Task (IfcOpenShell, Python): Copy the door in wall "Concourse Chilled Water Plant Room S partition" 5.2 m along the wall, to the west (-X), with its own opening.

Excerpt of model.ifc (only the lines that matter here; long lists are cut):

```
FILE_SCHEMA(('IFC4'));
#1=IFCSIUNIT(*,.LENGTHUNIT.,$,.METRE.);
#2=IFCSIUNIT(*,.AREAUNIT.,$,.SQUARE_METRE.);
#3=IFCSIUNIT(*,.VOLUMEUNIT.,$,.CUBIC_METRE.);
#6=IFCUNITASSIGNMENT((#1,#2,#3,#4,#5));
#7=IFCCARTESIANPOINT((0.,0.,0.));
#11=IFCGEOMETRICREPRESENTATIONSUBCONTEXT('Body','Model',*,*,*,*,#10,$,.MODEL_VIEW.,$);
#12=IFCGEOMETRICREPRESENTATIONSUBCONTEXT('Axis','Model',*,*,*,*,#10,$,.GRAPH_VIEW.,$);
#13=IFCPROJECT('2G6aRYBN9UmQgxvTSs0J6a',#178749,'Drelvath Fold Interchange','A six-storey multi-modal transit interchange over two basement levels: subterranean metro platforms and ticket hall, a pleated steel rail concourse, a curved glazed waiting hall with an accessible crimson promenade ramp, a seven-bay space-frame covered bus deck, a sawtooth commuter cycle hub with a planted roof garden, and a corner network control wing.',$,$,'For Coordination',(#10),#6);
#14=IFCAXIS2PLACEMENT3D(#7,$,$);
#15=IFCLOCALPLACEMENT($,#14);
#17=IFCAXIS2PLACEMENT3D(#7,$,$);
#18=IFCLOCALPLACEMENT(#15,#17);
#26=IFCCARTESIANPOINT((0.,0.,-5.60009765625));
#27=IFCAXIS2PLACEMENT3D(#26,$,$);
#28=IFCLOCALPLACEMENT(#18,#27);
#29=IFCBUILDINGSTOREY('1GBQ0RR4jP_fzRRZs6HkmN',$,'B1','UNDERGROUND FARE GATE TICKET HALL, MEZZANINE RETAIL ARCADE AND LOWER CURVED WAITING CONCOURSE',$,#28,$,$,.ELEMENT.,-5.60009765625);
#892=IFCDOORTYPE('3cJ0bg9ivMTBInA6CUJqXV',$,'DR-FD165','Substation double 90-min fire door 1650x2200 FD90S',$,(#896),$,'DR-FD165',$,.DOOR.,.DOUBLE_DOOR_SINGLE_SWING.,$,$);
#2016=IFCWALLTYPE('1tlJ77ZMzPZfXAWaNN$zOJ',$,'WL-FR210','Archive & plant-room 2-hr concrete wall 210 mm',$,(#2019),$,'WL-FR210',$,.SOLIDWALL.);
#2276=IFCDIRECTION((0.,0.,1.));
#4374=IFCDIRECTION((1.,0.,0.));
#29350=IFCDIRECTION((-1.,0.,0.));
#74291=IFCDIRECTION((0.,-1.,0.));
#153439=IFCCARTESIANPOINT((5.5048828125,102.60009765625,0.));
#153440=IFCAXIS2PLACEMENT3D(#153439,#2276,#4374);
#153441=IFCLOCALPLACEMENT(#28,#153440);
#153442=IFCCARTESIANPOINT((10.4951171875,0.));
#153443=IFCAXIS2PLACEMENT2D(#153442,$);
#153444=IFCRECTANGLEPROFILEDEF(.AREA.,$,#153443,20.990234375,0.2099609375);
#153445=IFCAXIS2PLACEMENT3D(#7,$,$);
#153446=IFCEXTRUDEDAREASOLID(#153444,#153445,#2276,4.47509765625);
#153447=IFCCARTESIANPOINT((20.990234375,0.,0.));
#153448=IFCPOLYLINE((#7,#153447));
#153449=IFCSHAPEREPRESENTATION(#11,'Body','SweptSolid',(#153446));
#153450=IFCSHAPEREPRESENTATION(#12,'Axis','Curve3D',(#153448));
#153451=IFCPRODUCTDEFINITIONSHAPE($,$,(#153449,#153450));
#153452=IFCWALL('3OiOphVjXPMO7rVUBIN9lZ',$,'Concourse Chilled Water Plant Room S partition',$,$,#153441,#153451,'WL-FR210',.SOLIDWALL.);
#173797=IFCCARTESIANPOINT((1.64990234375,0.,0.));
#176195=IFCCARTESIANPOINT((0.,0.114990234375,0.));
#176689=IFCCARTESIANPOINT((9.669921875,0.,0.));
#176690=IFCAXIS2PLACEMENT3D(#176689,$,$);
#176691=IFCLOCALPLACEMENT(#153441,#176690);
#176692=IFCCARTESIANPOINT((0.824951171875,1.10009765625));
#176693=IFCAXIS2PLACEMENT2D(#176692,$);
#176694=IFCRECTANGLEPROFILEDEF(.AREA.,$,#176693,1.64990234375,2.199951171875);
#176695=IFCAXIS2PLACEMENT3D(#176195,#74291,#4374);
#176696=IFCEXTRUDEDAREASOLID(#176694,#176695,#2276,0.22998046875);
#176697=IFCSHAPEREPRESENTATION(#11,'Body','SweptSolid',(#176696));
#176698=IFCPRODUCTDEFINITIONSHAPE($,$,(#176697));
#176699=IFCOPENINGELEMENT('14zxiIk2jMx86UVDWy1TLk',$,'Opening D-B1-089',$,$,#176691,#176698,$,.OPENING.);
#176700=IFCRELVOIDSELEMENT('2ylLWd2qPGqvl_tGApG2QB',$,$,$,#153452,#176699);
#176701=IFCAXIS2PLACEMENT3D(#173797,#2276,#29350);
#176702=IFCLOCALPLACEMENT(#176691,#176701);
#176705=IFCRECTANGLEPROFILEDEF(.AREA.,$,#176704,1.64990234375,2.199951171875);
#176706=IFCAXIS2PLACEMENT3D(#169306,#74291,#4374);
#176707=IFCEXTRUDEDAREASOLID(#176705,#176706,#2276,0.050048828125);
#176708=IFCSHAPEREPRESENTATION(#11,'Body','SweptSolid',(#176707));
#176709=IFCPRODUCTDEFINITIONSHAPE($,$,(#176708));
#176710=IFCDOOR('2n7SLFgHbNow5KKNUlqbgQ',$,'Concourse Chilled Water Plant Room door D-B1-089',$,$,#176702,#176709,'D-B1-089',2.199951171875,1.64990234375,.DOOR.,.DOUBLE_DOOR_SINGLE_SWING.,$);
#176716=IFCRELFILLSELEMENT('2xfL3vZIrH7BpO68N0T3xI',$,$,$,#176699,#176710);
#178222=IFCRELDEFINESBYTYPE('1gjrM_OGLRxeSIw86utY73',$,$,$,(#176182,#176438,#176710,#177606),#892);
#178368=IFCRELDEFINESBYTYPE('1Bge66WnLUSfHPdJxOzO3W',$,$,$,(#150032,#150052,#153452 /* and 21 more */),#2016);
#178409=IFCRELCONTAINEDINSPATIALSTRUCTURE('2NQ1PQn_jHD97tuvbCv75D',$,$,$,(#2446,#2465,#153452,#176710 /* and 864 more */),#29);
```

```python
import ifcopenshell
import ifcopenshell.api.feature
import ifcopenshell.api.geometry
import ifcopenshell.api.root
import ifcopenshell.geom
import ifcopenshell.util.element
import ifcopenshell.util.placement
import ifcopenshell.util.shape
import ifcopenshell.util.unit

model = ifcopenshell.open("model.ifc")
unit_scale = ifcopenshell.util.unit.calculate_unit_scale(model)
settings = ifcopenshell.geom.settings()


def volume(element):
    """Net volume in cubic metres, openings subtracted."""
    shape = ifcopenshell.geom.create_shape(settings, element)
    return ifcopenshell.util.shape.get_volume(shape.geometry)


door = model.by_guid("2n7SLFgHbNow5KKNUlqbgQ")
opening = door.FillsVoids[0].RelatingOpeningElement
wall = opening.VoidsElements[0].RelatingBuildingElement
before = volume(wall)
shift = ifcopenshell.util.placement.get_local_placement(wall.ObjectPlacement)[:3, 0] * -5.2 / unit_scale

# copy_class copies the void relationship, type, container and properties, but no geometry.
new_opening = ifcopenshell.api.root.copy_class(model, product=opening)
new_opening.Representation = ifcopenshell.util.element.copy_deep(
    model, opening.Representation, exclude=["IfcGeometricRepresentationContext", "IfcRepresentationMap"]
)
new_door = ifcopenshell.api.root.copy_class(model, product=door)
new_door.Representation = ifcopenshell.util.element.copy_deep(
    model, door.Representation, exclude=["IfcGeometricRepresentationContext", "IfcRepresentationMap"]
)
new_door.Tag = None
ifcopenshell.api.feature.add_filling(model, opening=new_opening, element=new_door)

for old, new in ((opening, new_opening), (door, new_door)):
    matrix = ifcopenshell.util.placement.get_local_placement(old.ObjectPlacement)
    matrix[:3, 3] += shift
    ifcopenshell.api.geometry.edit_object_placement(model, product=new, matrix=matrix, is_si=False)

after = volume(wall)

print(f"wall volume {before:.3f} -> {after:.3f} m3")

model.write("model-out.ifc")
```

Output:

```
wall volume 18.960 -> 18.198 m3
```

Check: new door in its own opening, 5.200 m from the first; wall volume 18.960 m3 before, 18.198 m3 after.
